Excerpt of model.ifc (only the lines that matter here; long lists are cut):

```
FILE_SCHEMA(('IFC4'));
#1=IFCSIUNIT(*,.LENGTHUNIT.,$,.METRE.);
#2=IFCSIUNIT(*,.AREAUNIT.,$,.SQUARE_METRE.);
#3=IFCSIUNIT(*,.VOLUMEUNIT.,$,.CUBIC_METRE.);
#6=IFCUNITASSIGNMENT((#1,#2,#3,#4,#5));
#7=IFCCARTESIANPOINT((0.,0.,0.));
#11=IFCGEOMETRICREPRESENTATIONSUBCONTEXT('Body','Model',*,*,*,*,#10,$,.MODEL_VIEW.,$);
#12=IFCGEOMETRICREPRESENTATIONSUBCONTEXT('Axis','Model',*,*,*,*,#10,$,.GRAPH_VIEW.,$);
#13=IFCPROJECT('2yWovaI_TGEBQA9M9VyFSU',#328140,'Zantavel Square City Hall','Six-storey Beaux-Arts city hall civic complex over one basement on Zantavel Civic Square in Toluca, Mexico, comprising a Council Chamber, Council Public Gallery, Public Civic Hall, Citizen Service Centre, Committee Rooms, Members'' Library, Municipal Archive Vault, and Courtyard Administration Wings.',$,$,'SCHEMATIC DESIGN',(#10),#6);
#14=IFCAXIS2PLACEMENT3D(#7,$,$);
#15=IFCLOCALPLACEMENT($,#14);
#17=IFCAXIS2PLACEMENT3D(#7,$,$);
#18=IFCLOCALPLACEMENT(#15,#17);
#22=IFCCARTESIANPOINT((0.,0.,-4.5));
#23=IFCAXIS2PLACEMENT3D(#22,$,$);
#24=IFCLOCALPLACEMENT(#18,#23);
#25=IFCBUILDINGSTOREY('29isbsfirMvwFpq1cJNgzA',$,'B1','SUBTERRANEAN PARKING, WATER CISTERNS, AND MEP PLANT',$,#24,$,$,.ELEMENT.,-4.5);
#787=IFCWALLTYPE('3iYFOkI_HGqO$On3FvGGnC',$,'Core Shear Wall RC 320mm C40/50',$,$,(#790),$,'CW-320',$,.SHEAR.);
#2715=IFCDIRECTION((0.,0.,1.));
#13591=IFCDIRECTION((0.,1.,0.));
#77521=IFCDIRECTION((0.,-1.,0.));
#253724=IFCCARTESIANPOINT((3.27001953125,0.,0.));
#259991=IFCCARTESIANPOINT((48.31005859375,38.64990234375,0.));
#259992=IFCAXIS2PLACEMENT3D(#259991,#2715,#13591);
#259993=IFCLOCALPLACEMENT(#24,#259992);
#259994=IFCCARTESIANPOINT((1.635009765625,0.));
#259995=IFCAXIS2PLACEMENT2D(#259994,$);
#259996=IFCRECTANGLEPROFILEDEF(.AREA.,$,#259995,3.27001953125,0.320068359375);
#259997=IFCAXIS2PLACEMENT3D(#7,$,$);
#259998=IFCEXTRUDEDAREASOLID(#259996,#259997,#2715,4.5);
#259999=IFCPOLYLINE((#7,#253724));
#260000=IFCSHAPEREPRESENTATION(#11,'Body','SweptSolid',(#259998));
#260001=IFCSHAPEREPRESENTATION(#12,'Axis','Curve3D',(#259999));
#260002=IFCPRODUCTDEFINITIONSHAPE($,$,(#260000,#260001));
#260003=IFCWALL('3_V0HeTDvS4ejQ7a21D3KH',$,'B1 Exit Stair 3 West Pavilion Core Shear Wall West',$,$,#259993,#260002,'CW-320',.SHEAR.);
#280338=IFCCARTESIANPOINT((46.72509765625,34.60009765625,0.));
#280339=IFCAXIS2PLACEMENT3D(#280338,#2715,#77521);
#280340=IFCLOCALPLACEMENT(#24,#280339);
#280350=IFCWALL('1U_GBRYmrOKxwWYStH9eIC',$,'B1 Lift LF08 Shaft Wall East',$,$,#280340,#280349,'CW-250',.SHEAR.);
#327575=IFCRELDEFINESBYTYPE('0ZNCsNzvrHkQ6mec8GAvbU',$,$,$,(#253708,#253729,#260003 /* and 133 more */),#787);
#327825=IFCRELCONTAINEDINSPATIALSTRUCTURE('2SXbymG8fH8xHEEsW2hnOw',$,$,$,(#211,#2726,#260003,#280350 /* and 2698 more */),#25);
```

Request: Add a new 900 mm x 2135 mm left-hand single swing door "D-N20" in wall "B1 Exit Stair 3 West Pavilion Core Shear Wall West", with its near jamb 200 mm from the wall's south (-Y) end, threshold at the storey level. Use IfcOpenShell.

```python
import numpy as np
import ifcopenshell
import ifcopenshell.api.feature
import ifcopenshell.api.geometry
import ifcopenshell.api.root
import ifcopenshell.api.spatial
import ifcopenshell.geom
import ifcopenshell.util.element
import ifcopenshell.util.placement
import ifcopenshell.util.representation
import ifcopenshell.util.shape
import ifcopenshell.util.unit

model = ifcopenshell.open("model.ifc")
unit_scale = ifcopenshell.util.unit.calculate_unit_scale(model)
settings = ifcopenshell.geom.settings()


def volume(element):
    """Net volume in cubic metres, openings subtracted."""
    shape = ifcopenshell.geom.create_shape(settings, element)
    return ifcopenshell.util.shape.get_volume(shape.geometry)


wall = model.by_guid("3_V0HeTDvS4ejQ7a21D3KH")
storey = ifcopenshell.util.element.get_container(wall, ifc_class="IfcBuildingStorey")
context = ifcopenshell.util.representation.get_context(model, "Model", "Body", "MODEL_VIEW")
before = volume(wall)

width, height, from_end, sill = 0.9, 2.135, 0.2, 0.0  # metres

# The wall runs along its own X axis, and the end named is its -X end.
wall_shape = ifcopenshell.geom.create_shape(settings, wall)
x, y, z = ifcopenshell.util.shape.get_vertices(wall_shape.geometry).T
start = x.min() + from_end
face, thickness = float(y.min()), float(y.max() - y.min())
wall_matrix = ifcopenshell.util.placement.get_local_placement(wall.ObjectPlacement)
level = ifcopenshell.util.placement.get_local_placement(storey.ObjectPlacement)[2, 3]


def in_wall(x, y):
    """Placement at x, y metres in the wall's axes, at sill height."""
    matrix = wall_matrix.copy()
    matrix[:, 3] = wall_matrix @ np.array([x / unit_scale, y / unit_scale, 0.0, 1.0])
    matrix[2, 3] = level + sill / unit_scale
    return matrix


# Opening: a box that overshoots both wall faces by 50 mm.
opening = ifcopenshell.api.root.create_entity(model, ifc_class="IfcOpeningElement", predefined_type="OPENING")
box = ifcopenshell.api.geometry.add_wall_representation(
    model, context=context, length=width, height=height, thickness=thickness + 0.1
)
ifcopenshell.api.geometry.assign_representation(model, product=opening, representation=box)
ifcopenshell.api.geometry.edit_object_placement(model, product=opening, matrix=in_wall(start, face - 0.05), is_si=False)
ifcopenshell.api.feature.add_feature(model, feature=opening, element=wall)

door = ifcopenshell.api.root.create_entity(model, ifc_class="IfcDoor", name="D-N20", predefined_type="DOOR")
door.OverallWidth, door.OverallHeight = width / unit_scale, height / unit_scale
door.OperationType = "SINGLE_SWING_LEFT"
body = ifcopenshell.api.geometry.add_door_representation(
    model,
    context=context,
    overall_width=door.OverallWidth,
    overall_height=door.OverallHeight,
    operation_type="SINGLE_SWING_LEFT",
    lining_properties={"LiningDepth": thickness / unit_scale, "ThresholdDepth": thickness / unit_scale},
)
ifcopenshell.api.geometry.assign_representation(model, product=door, representation=body)
ifcopenshell.api.spatial.assign_container(model, products=[door], relating_structure=storey)
ifcopenshell.api.feature.add_filling(model, opening=opening, element=door)

# The lining spans the wall, so the door starts at the wall face.
ifcopenshell.api.geometry.edit_object_placement(model, product=door, matrix=in_wall(start, face), is_si=False)

after = volume(wall)

print(f"wall volume {before:.3f} -> {after:.3f} m3")

model.write("model-out.ifc")
```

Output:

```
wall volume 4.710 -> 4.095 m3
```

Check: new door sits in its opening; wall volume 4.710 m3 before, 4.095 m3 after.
